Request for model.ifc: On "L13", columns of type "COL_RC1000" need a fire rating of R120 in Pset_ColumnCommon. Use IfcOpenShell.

First a look at what the model holds.

```python
import ifcopenshell
import ifcopenshell.util.element

model = ifcopenshell.open("model.ifc")
print(model.schema)
storey = next(s for s in model.by_type("IfcBuildingStorey") if s.Name == "L13")
columns = [e for e in ifcopenshell.util.element.get_decomposition(storey) if e.is_a("IfcColumn")]
seen = {}
for e in columns:
    element_type = ifcopenshell.util.element.get_type(e)
    key = (element_type.Name if element_type != e and element_type else None, ifcopenshell.util.element.get_pset(e, "Pset_ColumnCommon", "FireRating"))
    seen[key] = seen.get(key, 0) + 1
for (name, value), count in sorted(seen.items(), key=str):
    print(count, "x", name, "|", value)
```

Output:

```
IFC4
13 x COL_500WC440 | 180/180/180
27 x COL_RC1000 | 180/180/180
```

```python
import ifcopenshell
import ifcopenshell.api.pset
import ifcopenshell.util.element

model = ifcopenshell.open("model.ifc")

storey = next(s for s in model.by_type("IfcBuildingStorey") if s.Name == "L13")
columns = [e for e in ifcopenshell.util.element.get_decomposition(storey) if e.is_a("IfcColumn")]

count = 0
for e in columns:
    element_type = ifcopenshell.util.element.get_type(e)
    if element_type in (None, e) or element_type.Name != "COL_RC1000":
        continue
    found = ifcopenshell.util.element.get_pset(e, "Pset_ColumnCommon", should_inherit=False)
    if found:
        pset = model.by_id(found["id"])
        if len(ifcopenshell.util.element.get_elements_by_pset(pset)) > 1:
            pset = ifcopenshell.api.pset.unshare_pset(model, products=[e], pset=pset)[0]
    else:
        pset = ifcopenshell.api.pset.add_pset(model, product=e, name="Pset_ColumnCommon")
    ifcopenshell.api.pset.edit_pset(model, pset=pset, properties={"FireRating": "R120"})
    count += 1

print(count, "columns updated")

model.write("model_v2.ifc")
```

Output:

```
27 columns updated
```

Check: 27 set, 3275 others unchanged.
